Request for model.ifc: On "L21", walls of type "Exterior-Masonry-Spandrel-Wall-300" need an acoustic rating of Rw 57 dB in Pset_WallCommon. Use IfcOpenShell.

First a look at what the model holds.

```python
import ifcopenshell
import ifcopenshell.util.element

model = ifcopenshell.open("model.ifc")
print(model.schema)
storey = next(s for s in model.by_type("IfcBuildingStorey") if s.Name == "L21")
walls = [e for e in ifcopenshell.util.element.get_decomposition(storey) if e.is_a("IfcWall")]
seen = {}
for e in walls:
    element_type = ifcopenshell.util.element.get_type(e)
    key = (element_type.Name if element_type != e and element_type else None, ifcopenshell.util.element.get_pset(e, "Pset_WallCommon", "AcousticRating"))
    seen[key] = seen.get(key, 0) + 1
for (name, value), count in sorted(seen.items(), key=str):
    print(count, "x", name, "|", value)
```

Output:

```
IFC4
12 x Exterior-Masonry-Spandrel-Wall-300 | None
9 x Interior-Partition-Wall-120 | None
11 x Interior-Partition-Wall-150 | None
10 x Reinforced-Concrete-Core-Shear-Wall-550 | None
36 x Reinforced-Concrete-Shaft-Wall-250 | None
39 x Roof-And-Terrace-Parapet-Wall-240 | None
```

```python
import ifcopenshell
import ifcopenshell.api.pset
import ifcopenshell.util.element

model = ifcopenshell.open("model.ifc")

storey = next(s for s in model.by_type("IfcBuildingStorey") if s.Name == "L21")
walls = [e for e in ifcopenshell.util.element.get_decomposition(storey) if e.is_a("IfcWall")]

count = 0
for e in walls:
    element_type = ifcopenshell.util.element.get_type(e)
    if element_type in (None, e) or element_type.Name != "Exterior-Masonry-Spandrel-Wall-300":
        continue
    found = ifcopenshell.util.element.get_pset(e, "Pset_WallCommon", should_inherit=False)
    if found:
        pset = model.by_id(found["id"])
        if len(ifcopenshell.util.element.get_elements_by_pset(pset)) > 1:
            pset = ifcopenshell.api.pset.unshare_pset(model, products=[e], pset=pset)[0]
    else:
        pset = ifcopenshell.api.pset.add_pset(model, product=e, name="Pset_WallCommon")
    ifcopenshell.api.pset.edit_pset(model, pset=pset, properties={"AcousticRating": "Rw 57 dB"})
    count += 1

print(count, "walls updated")

model.write("model-out.ifc")
```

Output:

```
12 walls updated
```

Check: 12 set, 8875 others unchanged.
